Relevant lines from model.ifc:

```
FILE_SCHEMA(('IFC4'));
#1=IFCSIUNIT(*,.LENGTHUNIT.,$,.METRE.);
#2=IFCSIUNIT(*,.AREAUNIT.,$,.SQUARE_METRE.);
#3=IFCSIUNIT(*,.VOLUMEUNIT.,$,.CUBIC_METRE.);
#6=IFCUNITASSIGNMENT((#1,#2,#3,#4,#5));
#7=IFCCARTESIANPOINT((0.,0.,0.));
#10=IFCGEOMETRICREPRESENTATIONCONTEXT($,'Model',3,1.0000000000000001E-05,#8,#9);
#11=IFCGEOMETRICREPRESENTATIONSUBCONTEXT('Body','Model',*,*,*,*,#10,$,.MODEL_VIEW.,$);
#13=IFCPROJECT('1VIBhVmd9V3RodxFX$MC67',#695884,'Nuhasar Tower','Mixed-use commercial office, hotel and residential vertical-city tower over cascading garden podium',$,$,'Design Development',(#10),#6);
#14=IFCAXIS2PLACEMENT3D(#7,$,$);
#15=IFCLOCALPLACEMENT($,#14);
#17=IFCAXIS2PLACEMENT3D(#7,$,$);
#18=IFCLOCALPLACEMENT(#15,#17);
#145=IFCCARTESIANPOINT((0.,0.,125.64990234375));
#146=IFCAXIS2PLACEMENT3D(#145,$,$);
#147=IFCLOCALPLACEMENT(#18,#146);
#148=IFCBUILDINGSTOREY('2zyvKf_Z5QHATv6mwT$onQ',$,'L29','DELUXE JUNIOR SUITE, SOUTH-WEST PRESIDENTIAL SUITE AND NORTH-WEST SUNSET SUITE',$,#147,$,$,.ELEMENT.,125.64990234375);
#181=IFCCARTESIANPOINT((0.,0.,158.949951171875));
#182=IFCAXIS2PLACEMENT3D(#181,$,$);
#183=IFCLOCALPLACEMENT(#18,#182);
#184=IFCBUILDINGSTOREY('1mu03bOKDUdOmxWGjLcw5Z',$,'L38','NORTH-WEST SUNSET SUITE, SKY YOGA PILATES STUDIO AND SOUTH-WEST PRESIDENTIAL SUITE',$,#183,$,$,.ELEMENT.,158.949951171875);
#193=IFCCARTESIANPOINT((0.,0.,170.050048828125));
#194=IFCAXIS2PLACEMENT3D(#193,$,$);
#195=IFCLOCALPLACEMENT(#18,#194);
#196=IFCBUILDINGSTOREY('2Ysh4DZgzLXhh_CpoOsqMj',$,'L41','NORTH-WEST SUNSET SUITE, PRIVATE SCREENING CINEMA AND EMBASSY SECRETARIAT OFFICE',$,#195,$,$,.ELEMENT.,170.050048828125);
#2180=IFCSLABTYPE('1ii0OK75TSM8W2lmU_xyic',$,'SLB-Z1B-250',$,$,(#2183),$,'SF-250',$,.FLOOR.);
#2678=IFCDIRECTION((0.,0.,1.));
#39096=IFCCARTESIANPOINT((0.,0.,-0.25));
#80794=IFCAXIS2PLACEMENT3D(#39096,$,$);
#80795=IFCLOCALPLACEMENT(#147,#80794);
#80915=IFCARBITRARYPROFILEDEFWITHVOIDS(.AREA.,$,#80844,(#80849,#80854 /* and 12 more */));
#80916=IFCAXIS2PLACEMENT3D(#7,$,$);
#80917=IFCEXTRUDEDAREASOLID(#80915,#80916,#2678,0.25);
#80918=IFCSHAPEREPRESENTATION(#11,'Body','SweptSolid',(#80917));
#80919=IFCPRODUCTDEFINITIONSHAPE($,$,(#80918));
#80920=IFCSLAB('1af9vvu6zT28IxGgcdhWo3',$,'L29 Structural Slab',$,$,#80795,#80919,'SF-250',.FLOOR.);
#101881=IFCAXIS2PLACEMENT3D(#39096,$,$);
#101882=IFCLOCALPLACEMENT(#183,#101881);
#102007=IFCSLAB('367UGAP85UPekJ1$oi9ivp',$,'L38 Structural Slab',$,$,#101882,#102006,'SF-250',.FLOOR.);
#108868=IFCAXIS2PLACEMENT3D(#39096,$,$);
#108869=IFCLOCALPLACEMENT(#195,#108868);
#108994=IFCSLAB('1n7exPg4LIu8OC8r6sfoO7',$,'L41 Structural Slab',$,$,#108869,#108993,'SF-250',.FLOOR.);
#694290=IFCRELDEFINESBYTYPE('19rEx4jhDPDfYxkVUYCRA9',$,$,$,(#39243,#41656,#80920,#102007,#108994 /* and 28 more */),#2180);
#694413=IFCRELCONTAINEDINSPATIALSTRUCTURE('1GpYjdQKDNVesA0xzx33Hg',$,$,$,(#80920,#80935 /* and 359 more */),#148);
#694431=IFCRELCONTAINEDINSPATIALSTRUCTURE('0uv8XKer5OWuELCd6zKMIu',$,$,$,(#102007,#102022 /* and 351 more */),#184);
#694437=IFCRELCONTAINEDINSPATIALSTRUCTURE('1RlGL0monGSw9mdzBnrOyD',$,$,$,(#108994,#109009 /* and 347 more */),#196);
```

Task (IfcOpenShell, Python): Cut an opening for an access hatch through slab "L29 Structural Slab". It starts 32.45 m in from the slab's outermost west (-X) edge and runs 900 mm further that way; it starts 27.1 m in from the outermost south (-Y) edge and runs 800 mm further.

```python
import numpy as np
import ifcopenshell
import ifcopenshell.api.feature
import ifcopenshell.api.geometry
import ifcopenshell.api.root
import ifcopenshell.geom
import ifcopenshell.util.placement
import ifcopenshell.util.representation
import ifcopenshell.util.shape
import ifcopenshell.util.unit

model = ifcopenshell.open("model.ifc")
unit_scale = ifcopenshell.util.unit.calculate_unit_scale(model)
settings = ifcopenshell.geom.settings()


def volume(element):
    """Net volume in cubic metres, openings subtracted."""
    shape = ifcopenshell.geom.create_shape(settings, element)
    return ifcopenshell.util.shape.get_volume(shape.geometry)


slab = model.by_guid("1af9vvu6zT28IxGgcdhWo3")
before = volume(slab)

# Extent in the slab's own axes, in metres. The edges named are its -X and -Y sides.
slab_shape = ifcopenshell.geom.create_shape(settings, slab)
vertices = ifcopenshell.util.shape.get_vertices(slab_shape.geometry)
x_min, y_min, bottom = vertices.min(axis=0)
top = vertices[:, 2].max()

opening = ifcopenshell.api.root.create_entity(model, ifc_class="IfcOpeningElement", name="Access hatch opening", predefined_type="OPENING")
context = ifcopenshell.util.representation.get_context(model, "Model", "Body", "MODEL_VIEW")
width, depth = 0.9, 0.8
outline = [(0.0, 0.0), (width, 0.0), (width, depth), (0.0, depth), (0.0, 0.0)]
# Overshoot both faces by 50 mm so the cut is clean.
shape = ifcopenshell.api.geometry.add_slab_representation(
    model, context=context, depth=top - bottom + 0.1, polyline=outline
)
ifcopenshell.api.geometry.assign_representation(model, product=opening, representation=shape)

matrix = ifcopenshell.util.placement.get_local_placement(slab.ObjectPlacement)
matrix[:, 3] = matrix @ np.append(np.array([x_min + 32.45, y_min + 27.1, bottom - 0.05]) / unit_scale, 1.0)
ifcopenshell.api.geometry.edit_object_placement(model, product=opening, matrix=matrix, is_si=False)
ifcopenshell.api.feature.add_feature(model, feature=opening, element=slab)

after = volume(slab)

print(f"slab volume {before:.3f} -> {after:.3f} m3")

model.write("model_updated.ifc")
```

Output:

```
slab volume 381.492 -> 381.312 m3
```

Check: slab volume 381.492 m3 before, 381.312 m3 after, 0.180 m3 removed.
